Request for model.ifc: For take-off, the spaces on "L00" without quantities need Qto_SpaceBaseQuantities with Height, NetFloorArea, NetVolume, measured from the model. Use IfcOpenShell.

First a look at what the model holds.

```python
import ifcopenshell
import ifcopenshell.util.element
import ifcopenshell.util.unit

model = ifcopenshell.open("model.ifc")
print(model.schema)
for unit_type in ("LENGTHUNIT", "AREAUNIT", "VOLUMEUNIT"):
    print(unit_type, ifcopenshell.util.unit.calculate_unit_scale(model, unit_type))
storey = next(s for s in model.by_type("IfcBuildingStorey") if s.Name == "L00")
spaces = [e for e in ifcopenshell.util.element.get_decomposition(storey) if e.is_a("IfcSpace")]
for e in sorted(spaces, key=lambda e: e.id()):
    print(e.id(), e.is_a(), e.Name, list(ifcopenshell.util.element.get_psets(e, qtos_only=True)), sep=" | ")
```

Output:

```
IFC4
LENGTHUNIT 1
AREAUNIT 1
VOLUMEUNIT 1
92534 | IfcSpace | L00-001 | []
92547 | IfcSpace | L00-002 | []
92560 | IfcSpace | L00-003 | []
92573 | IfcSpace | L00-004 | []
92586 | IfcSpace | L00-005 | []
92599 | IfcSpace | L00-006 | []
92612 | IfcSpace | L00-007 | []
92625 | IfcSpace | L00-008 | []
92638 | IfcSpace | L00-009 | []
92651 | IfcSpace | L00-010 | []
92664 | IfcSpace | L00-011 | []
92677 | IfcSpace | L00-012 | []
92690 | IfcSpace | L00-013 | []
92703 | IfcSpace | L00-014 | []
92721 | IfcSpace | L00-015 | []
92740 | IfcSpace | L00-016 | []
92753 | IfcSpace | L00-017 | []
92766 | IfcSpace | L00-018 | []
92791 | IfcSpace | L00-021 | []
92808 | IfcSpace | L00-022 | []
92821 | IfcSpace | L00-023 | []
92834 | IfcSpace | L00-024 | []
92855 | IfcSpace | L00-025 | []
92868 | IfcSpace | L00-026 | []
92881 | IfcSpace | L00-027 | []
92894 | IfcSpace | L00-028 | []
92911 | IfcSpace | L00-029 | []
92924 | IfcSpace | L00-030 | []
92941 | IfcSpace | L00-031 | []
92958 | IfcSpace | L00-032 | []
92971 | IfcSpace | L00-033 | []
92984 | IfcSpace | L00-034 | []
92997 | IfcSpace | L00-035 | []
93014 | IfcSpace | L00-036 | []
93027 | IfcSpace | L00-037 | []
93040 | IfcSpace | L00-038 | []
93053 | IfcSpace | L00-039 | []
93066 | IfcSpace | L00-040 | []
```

```python
import ifcopenshell
import ifcopenshell.api.pset
import ifcopenshell.geom
import ifcopenshell.util.element
import ifcopenshell.util.shape
import ifcopenshell.util.unit

model = ifcopenshell.open("model.ifc")
unit_scale = ifcopenshell.util.unit.calculate_unit_scale(model)
area_scale = ifcopenshell.util.unit.calculate_unit_scale(model, "AREAUNIT")
volume_scale = ifcopenshell.util.unit.calculate_unit_scale(model, "VOLUMEUNIT")
settings = ifcopenshell.geom.settings()

storey = next(s for s in model.by_type("IfcBuildingStorey") if s.Name == "L00")
spaces = [e for e in ifcopenshell.util.element.get_decomposition(storey) if e.is_a("IfcSpace")]

for e in sorted(spaces, key=lambda e: e.id()):
    if ifcopenshell.util.element.get_psets(e, qtos_only=True, should_inherit=False):
        continue
    # Geometry comes back in metres, in the element's own axes.
    shape = ifcopenshell.geom.create_shape(settings, e)
    values = {
        "Height": ifcopenshell.util.shape.get_z(shape.geometry) / unit_scale,
        "NetFloorArea": ifcopenshell.util.shape.get_footprint_area(shape.geometry) / area_scale,
        "NetVolume": ifcopenshell.util.shape.get_volume(shape.geometry) / volume_scale,
    }
    qto = ifcopenshell.api.pset.add_qto(model, product=e, name="Qto_SpaceBaseQuantities")
    ifcopenshell.api.pset.edit_qto(model, qto=qto, properties=values)
    print(e.id(), {k: round(v, 3) for k, v in values.items()})

model.write("model_updated.ifc")
```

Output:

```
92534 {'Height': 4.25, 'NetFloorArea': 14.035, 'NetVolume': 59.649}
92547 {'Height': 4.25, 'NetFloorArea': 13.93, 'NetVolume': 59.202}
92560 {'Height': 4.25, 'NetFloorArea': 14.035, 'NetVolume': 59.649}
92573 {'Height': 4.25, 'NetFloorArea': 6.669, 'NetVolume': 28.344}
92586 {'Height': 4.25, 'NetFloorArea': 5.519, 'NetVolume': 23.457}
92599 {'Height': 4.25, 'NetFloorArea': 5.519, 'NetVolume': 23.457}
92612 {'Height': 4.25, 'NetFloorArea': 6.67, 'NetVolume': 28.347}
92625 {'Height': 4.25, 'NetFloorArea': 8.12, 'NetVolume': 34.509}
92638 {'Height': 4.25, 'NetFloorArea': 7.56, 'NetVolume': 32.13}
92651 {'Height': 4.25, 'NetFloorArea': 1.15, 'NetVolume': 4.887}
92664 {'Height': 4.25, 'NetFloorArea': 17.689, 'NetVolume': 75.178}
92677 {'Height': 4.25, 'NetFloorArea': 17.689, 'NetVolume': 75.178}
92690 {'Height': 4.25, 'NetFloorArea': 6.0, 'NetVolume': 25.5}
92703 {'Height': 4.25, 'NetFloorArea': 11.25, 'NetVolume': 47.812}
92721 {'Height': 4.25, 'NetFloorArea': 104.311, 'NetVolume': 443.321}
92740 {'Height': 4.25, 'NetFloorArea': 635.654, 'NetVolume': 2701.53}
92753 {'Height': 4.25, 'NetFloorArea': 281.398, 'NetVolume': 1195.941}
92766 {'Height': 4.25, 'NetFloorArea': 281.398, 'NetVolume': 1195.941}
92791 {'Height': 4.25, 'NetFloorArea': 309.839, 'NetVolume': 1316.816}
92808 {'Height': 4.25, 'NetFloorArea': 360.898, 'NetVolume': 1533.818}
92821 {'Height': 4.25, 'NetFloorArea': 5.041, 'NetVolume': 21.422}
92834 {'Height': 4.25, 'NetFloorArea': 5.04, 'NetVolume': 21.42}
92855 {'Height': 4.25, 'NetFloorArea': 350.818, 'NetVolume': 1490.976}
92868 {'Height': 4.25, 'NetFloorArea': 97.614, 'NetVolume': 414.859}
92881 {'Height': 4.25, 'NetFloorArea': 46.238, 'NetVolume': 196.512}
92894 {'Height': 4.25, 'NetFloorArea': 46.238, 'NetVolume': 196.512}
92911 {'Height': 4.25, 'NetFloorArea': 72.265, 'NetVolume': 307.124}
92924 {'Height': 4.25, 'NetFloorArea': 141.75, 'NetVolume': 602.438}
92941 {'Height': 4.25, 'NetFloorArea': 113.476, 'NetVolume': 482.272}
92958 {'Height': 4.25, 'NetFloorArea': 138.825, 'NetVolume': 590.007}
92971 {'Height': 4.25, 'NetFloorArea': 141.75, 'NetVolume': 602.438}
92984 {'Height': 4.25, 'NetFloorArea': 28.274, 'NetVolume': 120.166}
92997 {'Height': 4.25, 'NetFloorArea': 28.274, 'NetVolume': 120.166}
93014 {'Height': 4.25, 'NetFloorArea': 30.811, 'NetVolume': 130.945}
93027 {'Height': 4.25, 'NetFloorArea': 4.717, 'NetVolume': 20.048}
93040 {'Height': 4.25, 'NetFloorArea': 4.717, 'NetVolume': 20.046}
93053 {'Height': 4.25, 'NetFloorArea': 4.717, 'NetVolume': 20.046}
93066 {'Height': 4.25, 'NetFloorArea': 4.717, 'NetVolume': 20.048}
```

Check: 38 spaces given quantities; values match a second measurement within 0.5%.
